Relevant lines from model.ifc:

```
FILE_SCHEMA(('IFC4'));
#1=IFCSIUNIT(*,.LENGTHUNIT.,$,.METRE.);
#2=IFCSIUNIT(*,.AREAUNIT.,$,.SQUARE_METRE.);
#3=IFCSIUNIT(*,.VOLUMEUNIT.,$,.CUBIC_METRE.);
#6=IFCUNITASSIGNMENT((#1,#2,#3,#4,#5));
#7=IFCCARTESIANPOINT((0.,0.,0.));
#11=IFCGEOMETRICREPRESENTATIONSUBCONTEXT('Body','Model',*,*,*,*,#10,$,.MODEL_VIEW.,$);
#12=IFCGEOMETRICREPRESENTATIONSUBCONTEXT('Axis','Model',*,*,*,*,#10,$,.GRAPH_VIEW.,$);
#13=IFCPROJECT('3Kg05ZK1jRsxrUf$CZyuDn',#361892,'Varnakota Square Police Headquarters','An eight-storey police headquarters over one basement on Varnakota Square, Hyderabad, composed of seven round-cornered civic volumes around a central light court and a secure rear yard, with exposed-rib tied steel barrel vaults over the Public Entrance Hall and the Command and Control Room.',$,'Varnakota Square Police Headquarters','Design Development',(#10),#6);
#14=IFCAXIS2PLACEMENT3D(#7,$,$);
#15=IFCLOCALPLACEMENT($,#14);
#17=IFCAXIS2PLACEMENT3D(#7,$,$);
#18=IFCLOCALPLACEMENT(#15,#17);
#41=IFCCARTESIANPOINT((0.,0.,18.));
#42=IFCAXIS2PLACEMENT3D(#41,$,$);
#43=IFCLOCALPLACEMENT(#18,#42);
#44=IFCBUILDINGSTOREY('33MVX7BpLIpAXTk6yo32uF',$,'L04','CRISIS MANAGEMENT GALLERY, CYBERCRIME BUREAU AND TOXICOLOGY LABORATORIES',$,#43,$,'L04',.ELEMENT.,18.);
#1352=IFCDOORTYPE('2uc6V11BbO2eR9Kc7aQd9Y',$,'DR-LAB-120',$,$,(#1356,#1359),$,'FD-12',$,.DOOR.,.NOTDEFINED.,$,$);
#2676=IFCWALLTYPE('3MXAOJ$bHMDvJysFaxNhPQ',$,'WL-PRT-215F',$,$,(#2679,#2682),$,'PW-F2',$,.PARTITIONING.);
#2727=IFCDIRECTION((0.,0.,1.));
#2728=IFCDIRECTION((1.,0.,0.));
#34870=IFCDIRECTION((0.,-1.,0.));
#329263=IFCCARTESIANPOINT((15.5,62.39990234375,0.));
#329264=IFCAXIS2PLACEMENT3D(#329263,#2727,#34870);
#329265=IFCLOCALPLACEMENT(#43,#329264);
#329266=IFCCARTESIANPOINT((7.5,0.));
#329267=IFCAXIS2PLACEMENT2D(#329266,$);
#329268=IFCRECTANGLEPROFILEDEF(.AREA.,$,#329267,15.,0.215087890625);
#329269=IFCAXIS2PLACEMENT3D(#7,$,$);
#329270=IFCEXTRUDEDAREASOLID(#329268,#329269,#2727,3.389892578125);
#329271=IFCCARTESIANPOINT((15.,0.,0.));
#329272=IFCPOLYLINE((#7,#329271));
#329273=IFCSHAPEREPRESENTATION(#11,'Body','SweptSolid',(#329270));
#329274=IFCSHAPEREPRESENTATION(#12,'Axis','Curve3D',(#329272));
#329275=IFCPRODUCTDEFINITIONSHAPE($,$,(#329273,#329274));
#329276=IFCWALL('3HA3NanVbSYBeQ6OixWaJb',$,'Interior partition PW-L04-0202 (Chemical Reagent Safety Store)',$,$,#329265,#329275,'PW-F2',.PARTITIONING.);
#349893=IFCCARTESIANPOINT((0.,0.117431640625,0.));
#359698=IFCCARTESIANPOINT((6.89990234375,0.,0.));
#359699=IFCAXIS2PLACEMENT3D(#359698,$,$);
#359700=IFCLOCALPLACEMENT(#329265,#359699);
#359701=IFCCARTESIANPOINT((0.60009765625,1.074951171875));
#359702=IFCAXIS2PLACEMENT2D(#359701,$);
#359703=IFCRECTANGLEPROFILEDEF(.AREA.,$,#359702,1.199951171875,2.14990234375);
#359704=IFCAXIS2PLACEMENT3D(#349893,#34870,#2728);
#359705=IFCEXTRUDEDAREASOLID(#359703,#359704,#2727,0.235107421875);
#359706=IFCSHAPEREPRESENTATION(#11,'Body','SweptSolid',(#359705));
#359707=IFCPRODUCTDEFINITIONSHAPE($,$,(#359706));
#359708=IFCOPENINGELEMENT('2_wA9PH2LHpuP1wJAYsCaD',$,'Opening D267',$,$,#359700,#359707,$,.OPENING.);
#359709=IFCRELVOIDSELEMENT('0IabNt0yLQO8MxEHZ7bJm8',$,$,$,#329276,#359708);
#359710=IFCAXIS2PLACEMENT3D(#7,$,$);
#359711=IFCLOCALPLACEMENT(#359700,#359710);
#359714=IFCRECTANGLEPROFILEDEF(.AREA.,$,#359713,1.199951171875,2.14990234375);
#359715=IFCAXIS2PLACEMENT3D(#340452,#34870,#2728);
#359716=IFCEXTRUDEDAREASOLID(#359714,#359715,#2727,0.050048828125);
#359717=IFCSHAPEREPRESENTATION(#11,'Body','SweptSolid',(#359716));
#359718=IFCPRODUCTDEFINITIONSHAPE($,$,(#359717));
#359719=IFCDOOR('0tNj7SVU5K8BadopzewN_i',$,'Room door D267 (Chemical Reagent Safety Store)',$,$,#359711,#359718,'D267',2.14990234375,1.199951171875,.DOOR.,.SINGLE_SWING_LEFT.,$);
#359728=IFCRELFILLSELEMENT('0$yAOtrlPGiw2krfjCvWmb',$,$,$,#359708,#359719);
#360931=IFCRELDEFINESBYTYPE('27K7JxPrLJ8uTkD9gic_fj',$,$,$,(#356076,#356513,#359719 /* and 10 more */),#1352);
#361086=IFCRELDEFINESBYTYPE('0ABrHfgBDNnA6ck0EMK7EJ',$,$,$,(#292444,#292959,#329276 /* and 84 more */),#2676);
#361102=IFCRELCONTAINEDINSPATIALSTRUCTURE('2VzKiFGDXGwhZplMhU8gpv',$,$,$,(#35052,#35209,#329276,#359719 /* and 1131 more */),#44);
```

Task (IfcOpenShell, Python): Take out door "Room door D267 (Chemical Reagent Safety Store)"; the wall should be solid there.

```python
import ifcopenshell
import ifcopenshell.api.feature
import ifcopenshell.api.root
import ifcopenshell.geom
import ifcopenshell.util.shape

model = ifcopenshell.open("model.ifc")
settings = ifcopenshell.geom.settings()


def volume(element):
    """Net volume in cubic metres, openings subtracted."""
    shape = ifcopenshell.geom.create_shape(settings, element)
    return ifcopenshell.util.shape.get_volume(shape.geometry)


door = model.by_guid("0tNj7SVU5K8BadopzewN_i")
opening = door.FillsVoids[0].RelatingOpeningElement
wall = opening.VoidsElements[0].RelatingBuildingElement
before = volume(wall)

ifcopenshell.api.root.remove_product(model, product=door)
ifcopenshell.api.feature.remove_feature(model, feature=opening)

after = volume(wall)

print(f"wall volume {before:.3f} -> {after:.3f} m3")

model.write("model_edited.ifc")
```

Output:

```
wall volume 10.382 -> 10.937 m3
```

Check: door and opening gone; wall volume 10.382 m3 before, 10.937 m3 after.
